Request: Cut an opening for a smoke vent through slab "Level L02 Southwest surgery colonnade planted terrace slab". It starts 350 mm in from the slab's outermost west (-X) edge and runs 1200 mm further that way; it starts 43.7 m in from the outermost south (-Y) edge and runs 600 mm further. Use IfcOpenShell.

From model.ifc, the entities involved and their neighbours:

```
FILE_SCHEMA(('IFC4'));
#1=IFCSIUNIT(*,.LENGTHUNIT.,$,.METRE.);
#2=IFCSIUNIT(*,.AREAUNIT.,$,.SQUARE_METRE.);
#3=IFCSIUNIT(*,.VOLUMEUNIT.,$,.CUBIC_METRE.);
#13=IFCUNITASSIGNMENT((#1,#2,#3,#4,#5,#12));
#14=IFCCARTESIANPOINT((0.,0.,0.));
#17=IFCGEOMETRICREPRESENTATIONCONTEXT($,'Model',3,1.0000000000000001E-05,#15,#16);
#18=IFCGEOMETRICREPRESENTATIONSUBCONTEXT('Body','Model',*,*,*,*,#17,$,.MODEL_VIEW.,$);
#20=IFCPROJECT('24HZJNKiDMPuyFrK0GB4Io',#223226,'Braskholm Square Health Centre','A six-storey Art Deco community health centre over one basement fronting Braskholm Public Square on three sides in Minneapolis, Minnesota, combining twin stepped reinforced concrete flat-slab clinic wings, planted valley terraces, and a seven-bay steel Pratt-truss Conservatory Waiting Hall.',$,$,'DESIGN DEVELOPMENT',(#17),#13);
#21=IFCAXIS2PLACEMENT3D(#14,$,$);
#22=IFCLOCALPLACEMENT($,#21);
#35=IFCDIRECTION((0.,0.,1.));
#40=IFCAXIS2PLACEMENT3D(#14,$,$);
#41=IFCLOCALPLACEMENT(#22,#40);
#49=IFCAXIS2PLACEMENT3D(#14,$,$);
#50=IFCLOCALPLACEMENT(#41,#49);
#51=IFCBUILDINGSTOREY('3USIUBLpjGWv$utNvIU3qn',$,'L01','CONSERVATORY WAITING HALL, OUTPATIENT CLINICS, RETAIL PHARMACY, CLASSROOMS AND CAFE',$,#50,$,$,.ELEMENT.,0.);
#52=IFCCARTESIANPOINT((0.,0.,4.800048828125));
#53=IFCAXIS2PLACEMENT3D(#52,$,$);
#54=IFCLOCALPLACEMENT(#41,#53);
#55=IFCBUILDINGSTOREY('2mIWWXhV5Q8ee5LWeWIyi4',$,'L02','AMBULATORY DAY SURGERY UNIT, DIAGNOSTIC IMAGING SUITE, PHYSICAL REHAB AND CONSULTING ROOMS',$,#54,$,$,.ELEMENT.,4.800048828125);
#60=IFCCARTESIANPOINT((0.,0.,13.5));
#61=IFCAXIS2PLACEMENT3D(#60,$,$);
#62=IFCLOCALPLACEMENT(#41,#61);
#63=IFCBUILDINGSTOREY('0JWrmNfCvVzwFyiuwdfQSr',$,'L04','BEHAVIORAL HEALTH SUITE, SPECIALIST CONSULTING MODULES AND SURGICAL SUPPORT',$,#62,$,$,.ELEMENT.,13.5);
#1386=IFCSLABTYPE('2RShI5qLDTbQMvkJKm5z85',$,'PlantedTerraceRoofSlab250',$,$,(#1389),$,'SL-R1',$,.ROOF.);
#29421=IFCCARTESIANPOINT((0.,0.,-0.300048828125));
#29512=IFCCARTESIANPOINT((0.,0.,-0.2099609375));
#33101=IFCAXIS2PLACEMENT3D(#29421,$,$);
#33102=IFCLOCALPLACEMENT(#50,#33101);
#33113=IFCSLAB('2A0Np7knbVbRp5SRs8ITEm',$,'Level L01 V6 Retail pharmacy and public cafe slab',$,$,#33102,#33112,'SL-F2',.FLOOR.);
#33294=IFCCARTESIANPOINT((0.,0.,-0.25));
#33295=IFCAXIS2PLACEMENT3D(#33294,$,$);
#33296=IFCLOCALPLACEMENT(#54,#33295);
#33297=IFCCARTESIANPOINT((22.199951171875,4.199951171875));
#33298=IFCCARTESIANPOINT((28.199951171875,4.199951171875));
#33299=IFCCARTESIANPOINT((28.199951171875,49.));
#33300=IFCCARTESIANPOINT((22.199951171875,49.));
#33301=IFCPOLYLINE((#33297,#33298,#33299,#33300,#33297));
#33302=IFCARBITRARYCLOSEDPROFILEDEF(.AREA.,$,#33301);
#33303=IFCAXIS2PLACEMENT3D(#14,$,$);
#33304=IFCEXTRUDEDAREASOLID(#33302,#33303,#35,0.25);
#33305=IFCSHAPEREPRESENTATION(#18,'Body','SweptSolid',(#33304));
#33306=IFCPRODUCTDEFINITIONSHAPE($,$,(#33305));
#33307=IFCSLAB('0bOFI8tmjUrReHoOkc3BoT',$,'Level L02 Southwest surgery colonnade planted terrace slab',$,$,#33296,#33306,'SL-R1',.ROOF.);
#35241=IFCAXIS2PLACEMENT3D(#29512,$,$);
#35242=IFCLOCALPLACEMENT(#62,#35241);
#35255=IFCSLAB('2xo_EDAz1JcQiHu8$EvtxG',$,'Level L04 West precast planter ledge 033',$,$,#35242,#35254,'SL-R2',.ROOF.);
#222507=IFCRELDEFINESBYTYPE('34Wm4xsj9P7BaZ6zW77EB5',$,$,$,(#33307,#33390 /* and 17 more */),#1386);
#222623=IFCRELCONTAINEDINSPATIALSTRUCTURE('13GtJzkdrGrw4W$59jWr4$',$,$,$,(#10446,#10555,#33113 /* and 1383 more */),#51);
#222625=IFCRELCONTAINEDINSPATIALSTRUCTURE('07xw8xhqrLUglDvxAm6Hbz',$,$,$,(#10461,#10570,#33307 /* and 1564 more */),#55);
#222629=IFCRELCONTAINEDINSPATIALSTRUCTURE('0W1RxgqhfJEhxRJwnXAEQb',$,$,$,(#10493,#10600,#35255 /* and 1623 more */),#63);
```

```python
import numpy as np
import ifcopenshell
import ifcopenshell.api.feature
import ifcopenshell.api.geometry
import ifcopenshell.api.root
import ifcopenshell.geom
import ifcopenshell.util.placement
import ifcopenshell.util.representation
import ifcopenshell.util.shape
import ifcopenshell.util.unit

model = ifcopenshell.open("model.ifc")
unit_scale = ifcopenshell.util.unit.calculate_unit_scale(model)
settings = ifcopenshell.geom.settings()


def volume(element):
    """Net volume in cubic metres, openings subtracted."""
    shape = ifcopenshell.geom.create_shape(settings, element)
    return ifcopenshell.util.shape.get_volume(shape.geometry)


slab = model.by_guid("0bOFI8tmjUrReHoOkc3BoT")
before = volume(slab)

# Extent in the slab's own axes, in metres. The edges named are its -X and -Y sides.
slab_shape = ifcopenshell.geom.create_shape(settings, slab)
vertices = ifcopenshell.util.shape.get_vertices(slab_shape.geometry)
x_min, y_min, bottom = vertices.min(axis=0)
top = vertices[:, 2].max()

opening = ifcopenshell.api.root.create_entity(model, ifc_class="IfcOpeningElement", name="Smoke vent opening", predefined_type="OPENING")
context = ifcopenshell.util.representation.get_context(model, "Model", "Body", "MODEL_VIEW")
width, depth = 1.2, 0.6
outline = [(0.0, 0.0), (width, 0.0), (width, depth), (0.0, depth), (0.0, 0.0)]
# Overshoot both faces by 50 mm so the cut is clean.
shape = ifcopenshell.api.geometry.add_slab_representation(
    model, context=context, depth=top - bottom + 0.1, polyline=outline
)
ifcopenshell.api.geometry.assign_representation(model, product=opening, representation=shape)

matrix = ifcopenshell.util.placement.get_local_placement(slab.ObjectPlacement)
matrix[:, 3] = matrix @ np.append(np.array([x_min + 0.35, y_min + 43.7, bottom - 0.05]) / unit_scale, 1.0)
ifcopenshell.api.geometry.edit_object_placement(model, product=opening, matrix=matrix, is_si=False)
ifcopenshell.api.feature.add_feature(model, feature=opening, element=slab)

after = volume(slab)

print(f"slab volume {before:.3f} -> {after:.3f} m3")

model.write("model_edited.ifc")
```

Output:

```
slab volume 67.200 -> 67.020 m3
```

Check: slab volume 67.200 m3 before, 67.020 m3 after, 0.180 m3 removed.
